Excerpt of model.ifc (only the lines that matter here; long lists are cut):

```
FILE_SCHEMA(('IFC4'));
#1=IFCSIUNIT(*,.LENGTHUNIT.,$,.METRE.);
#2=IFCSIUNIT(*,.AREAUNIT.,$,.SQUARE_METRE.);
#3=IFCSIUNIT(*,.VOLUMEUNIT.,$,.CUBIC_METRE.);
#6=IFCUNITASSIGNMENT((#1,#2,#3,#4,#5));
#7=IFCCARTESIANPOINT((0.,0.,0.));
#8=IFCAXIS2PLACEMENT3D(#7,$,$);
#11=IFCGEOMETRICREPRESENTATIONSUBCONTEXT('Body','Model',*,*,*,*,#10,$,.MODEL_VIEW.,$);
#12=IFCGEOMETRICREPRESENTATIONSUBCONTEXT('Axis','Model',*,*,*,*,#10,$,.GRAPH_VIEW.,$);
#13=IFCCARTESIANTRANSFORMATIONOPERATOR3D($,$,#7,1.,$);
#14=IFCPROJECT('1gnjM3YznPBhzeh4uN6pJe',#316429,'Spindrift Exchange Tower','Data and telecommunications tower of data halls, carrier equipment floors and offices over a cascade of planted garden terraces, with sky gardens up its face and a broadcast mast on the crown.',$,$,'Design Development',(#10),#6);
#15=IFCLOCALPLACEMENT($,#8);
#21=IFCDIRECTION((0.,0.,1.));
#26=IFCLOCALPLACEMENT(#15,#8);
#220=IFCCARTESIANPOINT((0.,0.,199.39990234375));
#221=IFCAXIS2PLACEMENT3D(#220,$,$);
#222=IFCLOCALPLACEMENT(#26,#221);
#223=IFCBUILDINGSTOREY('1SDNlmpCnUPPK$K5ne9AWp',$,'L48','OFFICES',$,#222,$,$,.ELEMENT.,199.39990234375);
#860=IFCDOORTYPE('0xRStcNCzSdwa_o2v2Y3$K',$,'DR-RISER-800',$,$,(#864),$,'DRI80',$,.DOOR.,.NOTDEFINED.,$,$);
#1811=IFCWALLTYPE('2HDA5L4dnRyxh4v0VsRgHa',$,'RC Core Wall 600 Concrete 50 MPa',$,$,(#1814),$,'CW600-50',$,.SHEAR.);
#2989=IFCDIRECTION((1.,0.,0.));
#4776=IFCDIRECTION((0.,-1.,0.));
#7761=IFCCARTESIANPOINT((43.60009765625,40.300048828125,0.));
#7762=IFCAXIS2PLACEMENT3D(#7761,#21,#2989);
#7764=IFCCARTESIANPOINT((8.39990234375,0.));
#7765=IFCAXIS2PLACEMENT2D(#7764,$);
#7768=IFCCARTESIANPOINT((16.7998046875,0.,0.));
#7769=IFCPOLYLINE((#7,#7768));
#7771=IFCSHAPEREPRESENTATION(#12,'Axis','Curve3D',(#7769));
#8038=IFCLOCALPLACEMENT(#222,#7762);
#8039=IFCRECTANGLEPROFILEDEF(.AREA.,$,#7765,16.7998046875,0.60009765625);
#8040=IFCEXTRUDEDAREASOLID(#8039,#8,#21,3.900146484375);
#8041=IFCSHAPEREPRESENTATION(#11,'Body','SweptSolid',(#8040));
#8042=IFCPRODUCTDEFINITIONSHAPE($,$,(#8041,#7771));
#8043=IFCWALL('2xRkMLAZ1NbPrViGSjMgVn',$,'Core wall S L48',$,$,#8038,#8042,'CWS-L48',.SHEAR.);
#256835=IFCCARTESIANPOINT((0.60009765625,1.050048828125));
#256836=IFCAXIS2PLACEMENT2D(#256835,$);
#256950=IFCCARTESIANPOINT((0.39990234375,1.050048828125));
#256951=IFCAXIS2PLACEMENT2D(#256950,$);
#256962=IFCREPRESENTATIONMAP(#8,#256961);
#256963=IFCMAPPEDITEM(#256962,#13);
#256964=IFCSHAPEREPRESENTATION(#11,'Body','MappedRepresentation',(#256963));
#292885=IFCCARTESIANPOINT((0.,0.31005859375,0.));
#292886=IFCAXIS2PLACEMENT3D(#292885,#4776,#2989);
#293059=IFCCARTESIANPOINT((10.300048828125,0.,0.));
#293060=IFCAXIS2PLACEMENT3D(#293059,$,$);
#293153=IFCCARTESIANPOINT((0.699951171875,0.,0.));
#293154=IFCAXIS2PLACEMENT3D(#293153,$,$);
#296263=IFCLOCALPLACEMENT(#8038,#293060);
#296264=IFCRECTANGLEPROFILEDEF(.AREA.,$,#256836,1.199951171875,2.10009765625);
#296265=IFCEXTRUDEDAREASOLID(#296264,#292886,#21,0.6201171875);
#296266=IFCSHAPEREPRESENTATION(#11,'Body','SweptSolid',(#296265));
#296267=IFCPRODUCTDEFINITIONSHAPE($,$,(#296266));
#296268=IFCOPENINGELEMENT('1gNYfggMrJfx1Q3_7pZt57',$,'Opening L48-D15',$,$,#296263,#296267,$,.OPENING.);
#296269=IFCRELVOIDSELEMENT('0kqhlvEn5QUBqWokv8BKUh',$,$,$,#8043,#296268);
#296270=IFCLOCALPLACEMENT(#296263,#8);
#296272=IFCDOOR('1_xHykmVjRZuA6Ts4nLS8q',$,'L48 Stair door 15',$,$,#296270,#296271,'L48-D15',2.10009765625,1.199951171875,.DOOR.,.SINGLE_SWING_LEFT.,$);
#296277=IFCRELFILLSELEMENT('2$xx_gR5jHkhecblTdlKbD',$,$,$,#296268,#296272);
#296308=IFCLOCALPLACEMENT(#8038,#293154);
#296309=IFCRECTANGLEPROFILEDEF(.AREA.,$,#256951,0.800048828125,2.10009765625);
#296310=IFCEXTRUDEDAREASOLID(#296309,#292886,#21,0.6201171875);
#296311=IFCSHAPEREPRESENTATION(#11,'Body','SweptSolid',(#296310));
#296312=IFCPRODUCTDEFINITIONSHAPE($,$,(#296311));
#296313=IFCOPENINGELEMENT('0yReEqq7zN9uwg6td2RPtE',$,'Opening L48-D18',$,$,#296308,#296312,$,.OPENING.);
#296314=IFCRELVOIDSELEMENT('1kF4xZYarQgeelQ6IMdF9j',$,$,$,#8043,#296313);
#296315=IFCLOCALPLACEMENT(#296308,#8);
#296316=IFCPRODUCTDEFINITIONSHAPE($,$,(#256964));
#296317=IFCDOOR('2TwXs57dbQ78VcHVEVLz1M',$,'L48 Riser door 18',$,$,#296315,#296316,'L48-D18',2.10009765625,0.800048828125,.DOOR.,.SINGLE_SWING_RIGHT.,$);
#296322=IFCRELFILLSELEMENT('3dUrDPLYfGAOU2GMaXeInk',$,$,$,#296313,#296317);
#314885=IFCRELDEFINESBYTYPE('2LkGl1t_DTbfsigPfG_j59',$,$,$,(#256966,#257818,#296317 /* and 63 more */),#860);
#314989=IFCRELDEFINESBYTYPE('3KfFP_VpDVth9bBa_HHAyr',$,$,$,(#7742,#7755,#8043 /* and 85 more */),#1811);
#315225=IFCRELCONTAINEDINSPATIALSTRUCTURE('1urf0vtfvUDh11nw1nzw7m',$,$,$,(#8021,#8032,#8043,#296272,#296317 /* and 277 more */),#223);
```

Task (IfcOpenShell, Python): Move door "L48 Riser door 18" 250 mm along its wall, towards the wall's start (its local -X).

```python
import ifcopenshell
import ifcopenshell.api.geometry
import ifcopenshell.util.placement

model = ifcopenshell.open("model.ifc")

door = model.by_guid("2TwXs57dbQ78VcHVEVLz1M")
opening = door.FillsVoids[0].RelatingOpeningElement
wall = opening.VoidsElements[0].RelatingBuildingElement

wall_matrix = ifcopenshell.util.placement.get_local_placement(wall.ObjectPlacement)
shift = wall_matrix[:3, 0] * -0.25
before = ifcopenshell.util.placement.get_local_placement(door.ObjectPlacement)[:3, 3].copy()

# The door is placed relative to its opening, so it follows when the opening moves.
matrix = ifcopenshell.util.placement.get_local_placement(opening.ObjectPlacement)
matrix[:3, 3] += shift
ifcopenshell.api.geometry.edit_object_placement(
    model, product=opening, matrix=matrix, is_si=False, should_transform_children=True
)

after = ifcopenshell.util.placement.get_local_placement(door.ObjectPlacement)[:3, 3]
print("door moved by", (after - before).round(3) + 0.0)

model.write("model_edited.ifc")
```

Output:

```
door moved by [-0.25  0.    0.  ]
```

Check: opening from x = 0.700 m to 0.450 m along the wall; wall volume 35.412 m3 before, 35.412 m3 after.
